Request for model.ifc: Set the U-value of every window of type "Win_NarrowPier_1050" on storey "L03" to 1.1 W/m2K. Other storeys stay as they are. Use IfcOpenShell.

First a look at what the model holds.

```python
import ifcopenshell
import ifcopenshell.util.element

model = ifcopenshell.open("model.ifc")
print(model.schema)
storey = next(s for s in model.by_type("IfcBuildingStorey") if s.Name == "L03")
windows = [e for e in ifcopenshell.util.element.get_decomposition(storey) if e.is_a("IfcWindow")]
seen = {}
for e in windows:
    element_type = ifcopenshell.util.element.get_type(e)
    key = (element_type.Name if element_type != e and element_type else None, ifcopenshell.util.element.get_pset(e, "Pset_WindowCommon", "ThermalTransmittance"))
    seen[key] = seen.get(key, 0) + 1
for (name, value), count in sorted(seen.items(), key=str):
    print(count, "x", name, "|", value)
```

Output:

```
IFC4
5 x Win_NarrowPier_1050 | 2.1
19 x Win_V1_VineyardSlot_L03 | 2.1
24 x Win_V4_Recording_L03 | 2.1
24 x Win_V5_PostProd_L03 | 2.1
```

```python
import ifcopenshell
import ifcopenshell.api.pset
import ifcopenshell.util.element

model = ifcopenshell.open("model.ifc")

storey = next(s for s in model.by_type("IfcBuildingStorey") if s.Name == "L03")
windows = [e for e in ifcopenshell.util.element.get_decomposition(storey) if e.is_a("IfcWindow")]

count = 0
for e in windows:
    element_type = ifcopenshell.util.element.get_type(e)
    if element_type in (None, e) or element_type.Name != "Win_NarrowPier_1050":
        continue
    # add_pset returns the element's existing set when there is one.
    pset = ifcopenshell.api.pset.add_pset(model, product=e, name="Pset_WindowCommon")
    ifcopenshell.api.pset.edit_pset(model, pset=pset, properties={"ThermalTransmittance": 1.1})
    count += 1

print(count, "windows updated")

model.write("model-out.ifc")
```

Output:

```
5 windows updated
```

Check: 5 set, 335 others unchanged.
